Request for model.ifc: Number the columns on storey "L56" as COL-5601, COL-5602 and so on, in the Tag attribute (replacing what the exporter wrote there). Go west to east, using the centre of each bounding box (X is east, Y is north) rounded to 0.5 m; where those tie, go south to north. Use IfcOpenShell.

First a look at what the model holds.

```python
import ifcopenshell
import ifcopenshell.util.element
import ifcopenshell.util.placement

model = ifcopenshell.open("model.ifc")
print(model.schema)
storey = next(s for s in model.by_type("IfcBuildingStorey") if s.Name == "L56")
columns = [e for e in ifcopenshell.util.element.get_decomposition(storey) if e.is_a("IfcColumn")]
for e in sorted(columns, key=lambda e: e.id()):
    origin = ifcopenshell.util.placement.get_local_placement(e.ObjectPlacement)[:3, 3]
    print(e.id(), e.Tag, e.Name, origin.round(2) + 0.0, sep=" | ")
```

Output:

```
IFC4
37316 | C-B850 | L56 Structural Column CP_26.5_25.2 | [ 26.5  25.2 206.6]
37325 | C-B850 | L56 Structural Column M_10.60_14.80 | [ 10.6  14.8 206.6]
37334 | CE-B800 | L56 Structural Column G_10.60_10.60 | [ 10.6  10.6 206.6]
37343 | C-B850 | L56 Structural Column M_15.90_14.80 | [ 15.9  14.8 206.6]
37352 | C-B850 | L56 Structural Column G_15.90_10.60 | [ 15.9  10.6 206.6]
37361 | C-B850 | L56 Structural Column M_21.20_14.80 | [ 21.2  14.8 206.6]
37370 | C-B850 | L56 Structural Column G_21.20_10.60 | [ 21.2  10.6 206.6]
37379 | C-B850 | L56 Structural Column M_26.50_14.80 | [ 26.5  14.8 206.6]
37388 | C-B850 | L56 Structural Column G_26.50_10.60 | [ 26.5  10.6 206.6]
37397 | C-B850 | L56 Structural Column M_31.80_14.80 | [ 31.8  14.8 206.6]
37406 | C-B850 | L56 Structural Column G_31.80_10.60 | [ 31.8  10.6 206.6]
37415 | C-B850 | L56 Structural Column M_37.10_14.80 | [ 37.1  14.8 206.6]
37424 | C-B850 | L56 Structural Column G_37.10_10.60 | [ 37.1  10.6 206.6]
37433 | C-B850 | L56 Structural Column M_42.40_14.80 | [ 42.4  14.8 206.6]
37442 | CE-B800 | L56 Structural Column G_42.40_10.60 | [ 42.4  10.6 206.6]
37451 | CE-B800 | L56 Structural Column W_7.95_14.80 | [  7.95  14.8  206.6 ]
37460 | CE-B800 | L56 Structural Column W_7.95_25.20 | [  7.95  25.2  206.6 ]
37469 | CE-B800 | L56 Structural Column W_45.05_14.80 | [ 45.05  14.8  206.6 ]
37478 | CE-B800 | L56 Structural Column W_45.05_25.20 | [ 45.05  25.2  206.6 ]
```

```python
import ifcopenshell
import ifcopenshell.geom
import ifcopenshell.util.element
import ifcopenshell.util.shape

model = ifcopenshell.open("model.ifc")
settings = ifcopenshell.geom.settings()
settings.set("use-world-coords", True)


def centre(element):
    shape = ifcopenshell.geom.create_shape(settings, element)
    return ifcopenshell.util.shape.get_bbox_centroid(shape.geometry)


storey = next(s for s in model.by_type("IfcBuildingStorey") if s.Name == "L56")
columns = [e for e in ifcopenshell.util.element.get_decomposition(storey) if e.is_a("IfcColumn")]

# Insertion points can sit at a corner or the storey origin, so sort by the geometry (in metres).
centres = {e: centre(e) for e in columns}
columns.sort(key=lambda e: (round(centres[e][0] / 0.5), centres[e][1]))

for i, e in enumerate(columns, start=1):
    number = f"COL-56{i:02d}"
    e.Tag = number
    print(e.id(), number)

model.write("model_edited.ifc")
```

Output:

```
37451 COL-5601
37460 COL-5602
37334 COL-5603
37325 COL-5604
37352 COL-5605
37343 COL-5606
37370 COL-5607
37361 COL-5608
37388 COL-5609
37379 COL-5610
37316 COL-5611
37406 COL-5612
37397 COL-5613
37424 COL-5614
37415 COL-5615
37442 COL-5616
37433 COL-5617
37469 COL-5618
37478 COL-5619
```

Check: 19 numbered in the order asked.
